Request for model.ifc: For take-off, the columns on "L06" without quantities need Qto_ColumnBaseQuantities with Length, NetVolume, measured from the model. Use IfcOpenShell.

First a look at what the model holds.

```python
import ifcopenshell
import ifcopenshell.util.element
import ifcopenshell.util.unit

model = ifcopenshell.open("model.ifc")
print(model.schema)
for unit_type in ("LENGTHUNIT", "AREAUNIT", "VOLUMEUNIT"):
    print(unit_type, ifcopenshell.util.unit.calculate_unit_scale(model, unit_type))
storey = next(s for s in model.by_type("IfcBuildingStorey") if s.Name == "L06")
columns = [e for e in ifcopenshell.util.element.get_decomposition(storey) if e.is_a("IfcColumn")]
for e in sorted(columns, key=lambda e: e.id()):
    print(e.id(), e.is_a(), e.Name, list(ifcopenshell.util.element.get_psets(e, qtos_only=True)), sep=" | ")
```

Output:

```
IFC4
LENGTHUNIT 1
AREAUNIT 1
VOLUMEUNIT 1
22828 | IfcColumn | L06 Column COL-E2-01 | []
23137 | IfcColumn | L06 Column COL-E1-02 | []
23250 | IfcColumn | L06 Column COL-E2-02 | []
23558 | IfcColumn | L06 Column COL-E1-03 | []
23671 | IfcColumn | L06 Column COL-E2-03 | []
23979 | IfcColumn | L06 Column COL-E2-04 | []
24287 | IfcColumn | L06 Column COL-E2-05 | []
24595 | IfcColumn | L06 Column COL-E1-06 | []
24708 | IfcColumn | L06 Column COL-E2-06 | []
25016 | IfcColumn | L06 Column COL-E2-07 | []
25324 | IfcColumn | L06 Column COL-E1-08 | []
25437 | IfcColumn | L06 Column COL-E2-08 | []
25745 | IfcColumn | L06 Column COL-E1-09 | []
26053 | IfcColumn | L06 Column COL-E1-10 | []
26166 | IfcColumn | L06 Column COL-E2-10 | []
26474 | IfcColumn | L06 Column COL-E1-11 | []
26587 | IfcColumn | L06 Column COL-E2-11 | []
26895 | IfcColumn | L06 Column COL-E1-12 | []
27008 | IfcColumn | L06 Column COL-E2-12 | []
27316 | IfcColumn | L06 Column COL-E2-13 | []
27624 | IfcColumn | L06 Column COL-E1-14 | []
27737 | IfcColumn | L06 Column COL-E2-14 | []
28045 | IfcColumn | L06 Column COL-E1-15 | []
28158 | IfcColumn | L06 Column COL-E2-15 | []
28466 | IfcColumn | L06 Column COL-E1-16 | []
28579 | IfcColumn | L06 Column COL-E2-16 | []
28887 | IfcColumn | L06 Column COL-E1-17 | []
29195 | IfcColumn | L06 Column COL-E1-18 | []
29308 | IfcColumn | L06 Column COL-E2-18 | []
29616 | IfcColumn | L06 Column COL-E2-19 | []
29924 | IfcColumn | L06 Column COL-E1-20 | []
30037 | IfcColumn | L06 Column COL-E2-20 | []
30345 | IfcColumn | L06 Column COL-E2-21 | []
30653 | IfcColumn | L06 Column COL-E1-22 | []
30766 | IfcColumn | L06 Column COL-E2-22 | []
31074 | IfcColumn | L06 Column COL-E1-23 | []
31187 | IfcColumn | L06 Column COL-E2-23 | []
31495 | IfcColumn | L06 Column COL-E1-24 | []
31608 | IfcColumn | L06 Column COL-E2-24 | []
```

```python
import ifcopenshell
import ifcopenshell.api.pset
import ifcopenshell.geom
import ifcopenshell.util.element
import ifcopenshell.util.shape
import ifcopenshell.util.unit

model = ifcopenshell.open("model.ifc")
unit_scale = ifcopenshell.util.unit.calculate_unit_scale(model)
volume_scale = ifcopenshell.util.unit.calculate_unit_scale(model, "VOLUMEUNIT")
settings = ifcopenshell.geom.settings()

storey = next(s for s in model.by_type("IfcBuildingStorey") if s.Name == "L06")
columns = [e for e in ifcopenshell.util.element.get_decomposition(storey) if e.is_a("IfcColumn")]

for e in sorted(columns, key=lambda e: e.id()):
    if ifcopenshell.util.element.get_psets(e, qtos_only=True, should_inherit=False):
        continue
    # Geometry comes back in metres, in the element's own axes.
    shape = ifcopenshell.geom.create_shape(settings, e)
    values = {
        "Length": ifcopenshell.util.shape.get_z(shape.geometry) / unit_scale,
        "NetVolume": ifcopenshell.util.shape.get_volume(shape.geometry) / volume_scale,
    }
    qto = ifcopenshell.api.pset.add_qto(model, product=e, name="Qto_ColumnBaseQuantities")
    ifcopenshell.api.pset.edit_qto(model, qto=qto, properties=values)
    print(e.id(), {k: round(v, 3) for k, v in values.items()})

model.write("model_edited.ifc")
```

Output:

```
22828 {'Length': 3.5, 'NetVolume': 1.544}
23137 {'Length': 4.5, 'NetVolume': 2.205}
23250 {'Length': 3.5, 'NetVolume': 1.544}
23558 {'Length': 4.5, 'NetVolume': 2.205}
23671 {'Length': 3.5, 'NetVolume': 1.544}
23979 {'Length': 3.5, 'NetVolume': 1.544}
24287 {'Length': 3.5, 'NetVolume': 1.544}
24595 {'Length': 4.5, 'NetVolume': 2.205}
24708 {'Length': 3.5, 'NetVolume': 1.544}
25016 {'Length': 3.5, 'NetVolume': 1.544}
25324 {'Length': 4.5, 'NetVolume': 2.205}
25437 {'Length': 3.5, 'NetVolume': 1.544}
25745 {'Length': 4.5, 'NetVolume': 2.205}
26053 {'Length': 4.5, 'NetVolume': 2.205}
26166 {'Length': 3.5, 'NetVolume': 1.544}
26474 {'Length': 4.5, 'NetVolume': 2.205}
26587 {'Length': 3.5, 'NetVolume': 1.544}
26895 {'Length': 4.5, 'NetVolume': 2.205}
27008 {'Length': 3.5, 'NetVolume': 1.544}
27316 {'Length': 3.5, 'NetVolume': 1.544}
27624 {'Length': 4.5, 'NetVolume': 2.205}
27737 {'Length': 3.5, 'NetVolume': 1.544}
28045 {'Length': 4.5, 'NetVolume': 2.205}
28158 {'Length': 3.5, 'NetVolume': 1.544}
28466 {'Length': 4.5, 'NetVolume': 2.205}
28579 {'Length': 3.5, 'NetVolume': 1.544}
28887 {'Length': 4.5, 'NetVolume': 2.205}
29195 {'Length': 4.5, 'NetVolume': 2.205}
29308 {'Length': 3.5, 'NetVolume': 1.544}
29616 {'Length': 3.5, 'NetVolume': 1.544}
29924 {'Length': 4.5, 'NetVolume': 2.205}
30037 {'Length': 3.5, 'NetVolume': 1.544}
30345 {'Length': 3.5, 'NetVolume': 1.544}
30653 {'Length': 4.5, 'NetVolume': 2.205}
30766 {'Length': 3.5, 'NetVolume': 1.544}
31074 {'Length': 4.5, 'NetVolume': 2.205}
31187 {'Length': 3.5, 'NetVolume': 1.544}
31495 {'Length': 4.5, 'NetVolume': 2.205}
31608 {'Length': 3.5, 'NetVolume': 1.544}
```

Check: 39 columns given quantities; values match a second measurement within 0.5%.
